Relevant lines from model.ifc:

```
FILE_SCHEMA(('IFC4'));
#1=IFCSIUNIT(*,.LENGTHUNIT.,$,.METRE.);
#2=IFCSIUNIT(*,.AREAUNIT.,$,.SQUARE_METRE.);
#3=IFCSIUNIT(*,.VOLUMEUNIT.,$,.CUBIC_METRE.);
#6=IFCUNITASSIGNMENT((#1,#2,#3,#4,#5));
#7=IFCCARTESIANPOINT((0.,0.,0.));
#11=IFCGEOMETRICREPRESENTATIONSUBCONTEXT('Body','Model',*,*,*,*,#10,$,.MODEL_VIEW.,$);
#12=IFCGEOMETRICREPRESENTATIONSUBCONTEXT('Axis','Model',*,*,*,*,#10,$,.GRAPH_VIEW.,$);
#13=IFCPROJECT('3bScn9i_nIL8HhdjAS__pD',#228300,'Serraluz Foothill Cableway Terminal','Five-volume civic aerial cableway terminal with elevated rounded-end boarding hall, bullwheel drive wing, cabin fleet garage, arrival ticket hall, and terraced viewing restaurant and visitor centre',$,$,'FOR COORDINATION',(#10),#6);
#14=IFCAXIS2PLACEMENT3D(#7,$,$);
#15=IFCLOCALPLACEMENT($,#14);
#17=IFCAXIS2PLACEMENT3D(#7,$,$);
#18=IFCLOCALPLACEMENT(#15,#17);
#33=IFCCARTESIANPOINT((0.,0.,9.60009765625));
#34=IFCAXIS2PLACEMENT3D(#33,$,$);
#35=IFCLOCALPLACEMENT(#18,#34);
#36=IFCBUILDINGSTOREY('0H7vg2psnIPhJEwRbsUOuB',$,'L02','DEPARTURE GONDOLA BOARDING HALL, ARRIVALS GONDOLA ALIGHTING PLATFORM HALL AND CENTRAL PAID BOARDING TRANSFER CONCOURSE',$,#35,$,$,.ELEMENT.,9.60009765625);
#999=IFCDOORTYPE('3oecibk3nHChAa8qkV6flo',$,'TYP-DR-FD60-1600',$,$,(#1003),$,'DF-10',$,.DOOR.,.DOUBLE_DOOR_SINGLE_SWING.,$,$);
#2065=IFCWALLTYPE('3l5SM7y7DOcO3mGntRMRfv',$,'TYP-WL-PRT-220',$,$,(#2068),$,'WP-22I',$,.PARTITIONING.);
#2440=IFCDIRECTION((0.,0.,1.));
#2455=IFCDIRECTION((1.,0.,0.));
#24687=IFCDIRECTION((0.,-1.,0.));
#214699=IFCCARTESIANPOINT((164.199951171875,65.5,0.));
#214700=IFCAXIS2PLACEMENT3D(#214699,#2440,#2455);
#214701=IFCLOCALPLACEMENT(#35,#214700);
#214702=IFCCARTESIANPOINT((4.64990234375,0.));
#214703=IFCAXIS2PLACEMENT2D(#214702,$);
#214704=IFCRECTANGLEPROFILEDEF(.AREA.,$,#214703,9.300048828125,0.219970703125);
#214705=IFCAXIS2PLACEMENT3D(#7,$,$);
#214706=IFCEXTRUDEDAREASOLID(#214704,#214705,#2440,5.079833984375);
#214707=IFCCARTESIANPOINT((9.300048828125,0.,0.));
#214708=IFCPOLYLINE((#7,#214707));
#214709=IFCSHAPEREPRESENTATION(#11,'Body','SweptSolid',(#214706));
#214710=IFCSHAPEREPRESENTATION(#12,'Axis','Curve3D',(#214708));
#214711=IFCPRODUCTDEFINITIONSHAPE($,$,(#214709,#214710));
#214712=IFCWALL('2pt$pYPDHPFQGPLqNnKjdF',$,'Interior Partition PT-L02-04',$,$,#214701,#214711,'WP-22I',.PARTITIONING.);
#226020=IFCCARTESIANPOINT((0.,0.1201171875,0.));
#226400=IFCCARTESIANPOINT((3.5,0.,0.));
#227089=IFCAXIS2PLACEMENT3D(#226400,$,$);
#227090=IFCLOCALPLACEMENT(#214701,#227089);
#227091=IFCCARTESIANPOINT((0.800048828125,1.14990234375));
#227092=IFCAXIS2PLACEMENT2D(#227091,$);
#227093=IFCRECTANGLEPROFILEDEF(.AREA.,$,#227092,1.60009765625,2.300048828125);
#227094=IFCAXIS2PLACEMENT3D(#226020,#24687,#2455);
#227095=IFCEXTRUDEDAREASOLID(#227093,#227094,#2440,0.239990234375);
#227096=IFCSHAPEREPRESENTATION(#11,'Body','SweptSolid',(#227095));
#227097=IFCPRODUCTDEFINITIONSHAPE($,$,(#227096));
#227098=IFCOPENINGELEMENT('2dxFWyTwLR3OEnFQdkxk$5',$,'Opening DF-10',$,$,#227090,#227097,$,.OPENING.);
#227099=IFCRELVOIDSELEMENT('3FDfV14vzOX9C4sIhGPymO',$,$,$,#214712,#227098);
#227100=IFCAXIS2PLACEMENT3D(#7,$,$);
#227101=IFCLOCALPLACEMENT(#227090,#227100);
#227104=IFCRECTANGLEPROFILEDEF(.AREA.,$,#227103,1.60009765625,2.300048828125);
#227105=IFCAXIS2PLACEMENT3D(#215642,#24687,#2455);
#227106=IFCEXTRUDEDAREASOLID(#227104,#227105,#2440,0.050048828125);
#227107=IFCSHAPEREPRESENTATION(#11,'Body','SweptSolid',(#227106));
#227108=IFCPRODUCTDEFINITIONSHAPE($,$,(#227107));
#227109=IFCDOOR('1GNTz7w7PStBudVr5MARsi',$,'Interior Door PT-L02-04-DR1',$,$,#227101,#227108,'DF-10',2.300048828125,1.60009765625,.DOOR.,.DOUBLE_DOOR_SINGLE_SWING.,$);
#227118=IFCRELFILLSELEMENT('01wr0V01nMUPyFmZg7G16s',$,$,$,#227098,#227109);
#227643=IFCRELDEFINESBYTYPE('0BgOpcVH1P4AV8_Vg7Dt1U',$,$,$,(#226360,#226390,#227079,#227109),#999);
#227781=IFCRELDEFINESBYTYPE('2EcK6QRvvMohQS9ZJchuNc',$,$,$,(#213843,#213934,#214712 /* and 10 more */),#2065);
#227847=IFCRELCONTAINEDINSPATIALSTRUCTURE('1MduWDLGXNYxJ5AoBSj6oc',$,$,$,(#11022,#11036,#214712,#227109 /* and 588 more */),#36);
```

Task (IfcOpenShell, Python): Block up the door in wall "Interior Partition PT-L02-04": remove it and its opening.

```python
import ifcopenshell
import ifcopenshell.api.feature
import ifcopenshell.api.root
import ifcopenshell.geom
import ifcopenshell.util.shape

model = ifcopenshell.open("model.ifc")
settings = ifcopenshell.geom.settings()


def volume(element):
    """Net volume in cubic metres, openings subtracted."""
    shape = ifcopenshell.geom.create_shape(settings, element)
    return ifcopenshell.util.shape.get_volume(shape.geometry)


door = model.by_guid("1GNTz7w7PStBudVr5MARsi")
opening = door.FillsVoids[0].RelatingOpeningElement
wall = opening.VoidsElements[0].RelatingBuildingElement
before = volume(wall)

ifcopenshell.api.root.remove_product(model, product=door)
ifcopenshell.api.feature.remove_feature(model, feature=opening)

after = volume(wall)

print(f"wall volume {before:.3f} -> {after:.3f} m3")

model.write("model_edited.ifc")
```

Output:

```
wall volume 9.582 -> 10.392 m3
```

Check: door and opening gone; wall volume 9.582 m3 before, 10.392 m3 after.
